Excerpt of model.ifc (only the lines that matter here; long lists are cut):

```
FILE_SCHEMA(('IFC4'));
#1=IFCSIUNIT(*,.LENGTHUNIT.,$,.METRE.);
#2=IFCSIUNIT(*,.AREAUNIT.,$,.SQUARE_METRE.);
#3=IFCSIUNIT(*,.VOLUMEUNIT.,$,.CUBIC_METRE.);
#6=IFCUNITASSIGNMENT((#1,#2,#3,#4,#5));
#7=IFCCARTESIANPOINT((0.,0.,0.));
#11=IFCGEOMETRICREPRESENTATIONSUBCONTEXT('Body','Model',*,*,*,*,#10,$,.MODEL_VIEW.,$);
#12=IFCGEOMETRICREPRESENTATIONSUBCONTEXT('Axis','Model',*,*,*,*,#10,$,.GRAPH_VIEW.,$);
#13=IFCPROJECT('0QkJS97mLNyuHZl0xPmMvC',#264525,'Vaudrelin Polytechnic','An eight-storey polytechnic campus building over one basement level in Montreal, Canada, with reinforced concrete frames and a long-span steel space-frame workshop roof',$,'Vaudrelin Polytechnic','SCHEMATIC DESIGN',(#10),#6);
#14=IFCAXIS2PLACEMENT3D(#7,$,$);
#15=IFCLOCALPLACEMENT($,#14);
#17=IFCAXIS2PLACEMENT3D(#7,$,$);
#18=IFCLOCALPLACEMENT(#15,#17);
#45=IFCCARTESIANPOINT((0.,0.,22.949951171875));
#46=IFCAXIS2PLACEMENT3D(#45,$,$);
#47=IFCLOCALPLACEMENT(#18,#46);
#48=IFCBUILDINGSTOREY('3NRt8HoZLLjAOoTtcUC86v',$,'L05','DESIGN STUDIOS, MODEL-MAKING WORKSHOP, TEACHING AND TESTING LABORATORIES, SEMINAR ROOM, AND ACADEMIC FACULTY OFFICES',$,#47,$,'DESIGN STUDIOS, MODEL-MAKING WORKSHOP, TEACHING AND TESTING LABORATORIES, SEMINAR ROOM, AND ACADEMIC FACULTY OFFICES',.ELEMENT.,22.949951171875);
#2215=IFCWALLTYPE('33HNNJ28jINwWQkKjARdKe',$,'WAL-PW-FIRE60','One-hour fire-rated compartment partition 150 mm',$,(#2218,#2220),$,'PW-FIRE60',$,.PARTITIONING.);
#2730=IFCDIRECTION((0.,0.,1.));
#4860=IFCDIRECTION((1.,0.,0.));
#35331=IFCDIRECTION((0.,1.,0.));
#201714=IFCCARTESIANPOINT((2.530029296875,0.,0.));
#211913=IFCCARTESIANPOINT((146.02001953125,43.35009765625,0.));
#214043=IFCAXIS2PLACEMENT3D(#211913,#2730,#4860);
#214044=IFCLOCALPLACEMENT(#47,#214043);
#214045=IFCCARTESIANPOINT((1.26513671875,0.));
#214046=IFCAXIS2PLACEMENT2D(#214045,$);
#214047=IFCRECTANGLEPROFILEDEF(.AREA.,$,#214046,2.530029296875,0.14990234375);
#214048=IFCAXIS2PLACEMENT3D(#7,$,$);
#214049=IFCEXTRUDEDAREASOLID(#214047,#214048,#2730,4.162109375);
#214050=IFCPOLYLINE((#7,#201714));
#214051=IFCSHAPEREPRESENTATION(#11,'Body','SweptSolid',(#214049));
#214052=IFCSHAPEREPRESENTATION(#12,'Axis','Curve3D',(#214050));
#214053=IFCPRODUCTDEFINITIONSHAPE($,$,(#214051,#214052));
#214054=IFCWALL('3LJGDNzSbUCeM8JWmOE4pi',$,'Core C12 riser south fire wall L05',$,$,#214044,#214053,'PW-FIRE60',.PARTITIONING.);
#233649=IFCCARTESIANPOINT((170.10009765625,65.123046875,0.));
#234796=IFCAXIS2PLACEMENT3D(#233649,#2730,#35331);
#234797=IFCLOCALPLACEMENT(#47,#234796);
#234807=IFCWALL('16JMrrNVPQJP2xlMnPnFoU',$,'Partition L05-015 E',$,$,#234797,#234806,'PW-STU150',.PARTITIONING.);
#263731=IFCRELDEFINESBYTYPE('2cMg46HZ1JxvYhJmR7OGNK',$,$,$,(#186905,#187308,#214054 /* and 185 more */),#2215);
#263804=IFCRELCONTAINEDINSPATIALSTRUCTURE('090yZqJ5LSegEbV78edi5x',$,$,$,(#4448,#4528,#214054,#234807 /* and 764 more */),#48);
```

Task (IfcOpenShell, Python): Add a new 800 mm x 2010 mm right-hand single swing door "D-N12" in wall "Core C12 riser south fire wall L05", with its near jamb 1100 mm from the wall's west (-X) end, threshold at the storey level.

```python
import numpy as np
import ifcopenshell
import ifcopenshell.api.feature
import ifcopenshell.api.geometry
import ifcopenshell.api.root
import ifcopenshell.api.spatial
import ifcopenshell.geom
import ifcopenshell.util.element
import ifcopenshell.util.placement
import ifcopenshell.util.representation
import ifcopenshell.util.shape
import ifcopenshell.util.unit

model = ifcopenshell.open("model.ifc")
unit_scale = ifcopenshell.util.unit.calculate_unit_scale(model)
settings = ifcopenshell.geom.settings()


def volume(element):
    """Net volume in cubic metres, openings subtracted."""
    shape = ifcopenshell.geom.create_shape(settings, element)
    return ifcopenshell.util.shape.get_volume(shape.geometry)


wall = model.by_guid("3LJGDNzSbUCeM8JWmOE4pi")
storey = ifcopenshell.util.element.get_container(wall, ifc_class="IfcBuildingStorey")
context = ifcopenshell.util.representation.get_context(model, "Model", "Body", "MODEL_VIEW")
before = volume(wall)

width, height, from_end, sill = 0.8, 2.01, 1.1, 0.0  # metres

# The wall runs along its own X axis, and the end named is its -X end.
wall_shape = ifcopenshell.geom.create_shape(settings, wall)
x, y, z = ifcopenshell.util.shape.get_vertices(wall_shape.geometry).T
start = x.min() + from_end
face, thickness = float(y.min()), float(y.max() - y.min())
wall_matrix = ifcopenshell.util.placement.get_local_placement(wall.ObjectPlacement)
level = ifcopenshell.util.placement.get_local_placement(storey.ObjectPlacement)[2, 3]


def in_wall(x, y):
    """Placement at x, y metres in the wall's axes, at sill height."""
    matrix = wall_matrix.copy()
    matrix[:, 3] = wall_matrix @ np.array([x / unit_scale, y / unit_scale, 0.0, 1.0])
    matrix[2, 3] = level + sill / unit_scale
    return matrix


# Opening: a box that overshoots both wall faces by 50 mm.
opening = ifcopenshell.api.root.create_entity(model, ifc_class="IfcOpeningElement", predefined_type="OPENING")
box = ifcopenshell.api.geometry.add_wall_representation(
    model, context=context, length=width, height=height, thickness=thickness + 0.1
)
ifcopenshell.api.geometry.assign_representation(model, product=opening, representation=box)
ifcopenshell.api.geometry.edit_object_placement(model, product=opening, matrix=in_wall(start, face - 0.05), is_si=False)
ifcopenshell.api.feature.add_feature(model, feature=opening, element=wall)

door = ifcopenshell.api.root.create_entity(model, ifc_class="IfcDoor", name="D-N12", predefined_type="DOOR")
door.OverallWidth, door.OverallHeight = width / unit_scale, height / unit_scale
door.OperationType = "SINGLE_SWING_RIGHT"
body = ifcopenshell.api.geometry.add_door_representation(
    model,
    context=context,
    overall_width=door.OverallWidth,
    overall_height=door.OverallHeight,
    operation_type="SINGLE_SWING_RIGHT",
    lining_properties={"LiningDepth": thickness / unit_scale, "ThresholdDepth": thickness / unit_scale},
)
ifcopenshell.api.geometry.assign_representation(model, product=door, representation=body)
ifcopenshell.api.spatial.assign_container(model, products=[door], relating_structure=storey)
ifcopenshell.api.feature.add_filling(model, opening=opening, element=door)

# The lining spans the wall, so the door starts at the wall face.
ifcopenshell.api.geometry.edit_object_placement(model, product=door, matrix=in_wall(start, face), is_si=False)

after = volume(wall)

print(f"wall volume {before:.3f} -> {after:.3f} m3")

model.write("model_rev.ifc")
```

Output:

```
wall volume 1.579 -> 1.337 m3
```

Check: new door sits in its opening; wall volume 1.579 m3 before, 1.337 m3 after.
